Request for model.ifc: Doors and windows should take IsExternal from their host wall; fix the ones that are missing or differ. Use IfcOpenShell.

First a look at what the model holds.

```python
import ifcopenshell
import ifcopenshell.util.element

model = ifcopenshell.open("model.ifc")
print(model.schema)
seen = {}
for e in model.by_type("IfcDoor") + model.by_type("IfcWindow"):
    if not e.FillsVoids:
        continue
    host = e.FillsVoids[0].RelatingOpeningElement.VoidsElements[0].RelatingBuildingElement
    own = ifcopenshell.util.element.get_pset(e, f"Pset_{e.is_a()[3:].removesuffix('StandardCase')}Common", "IsExternal")
    wall = ifcopenshell.util.element.get_pset(host, "Pset_WallCommon", "IsExternal")
    seen[e.is_a(), own, wall] = seen.get((e.is_a(), own, wall), 0) + 1
for (cls, own, wall), count in sorted(seen.items(), key=str):
    print(count, cls, "IsExternal:", own, "| host wall:", wall)
```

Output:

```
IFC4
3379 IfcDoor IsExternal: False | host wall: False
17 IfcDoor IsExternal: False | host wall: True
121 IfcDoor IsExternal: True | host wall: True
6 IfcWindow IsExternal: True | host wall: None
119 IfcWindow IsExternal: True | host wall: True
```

```python
import ifcopenshell
import ifcopenshell.api.pset
import ifcopenshell.util.element

model = ifcopenshell.open("model.ifc")

count = 0
for ifc_class, pset_name in (("IfcDoor", "Pset_DoorCommon"), ("IfcWindow", "Pset_WindowCommon")):
    for e in model.by_type(ifc_class):
        if not e.FillsVoids:
            continue
        host = e.FillsVoids[0].RelatingOpeningElement.VoidsElements[0].RelatingBuildingElement
        external = ifcopenshell.util.element.get_pset(host, "Pset_WallCommon", "IsExternal")
        if external is None or ifcopenshell.util.element.get_pset(e, pset_name, "IsExternal") == external:
            continue
        pset = ifcopenshell.api.pset.add_pset(model, product=e, name=pset_name)
        ifcopenshell.api.pset.edit_pset(model, pset=pset, properties={"IsExternal": external})
        count += 1

print(count, "updated")

model.write("model_rev.ifc")
```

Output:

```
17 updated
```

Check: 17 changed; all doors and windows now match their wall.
